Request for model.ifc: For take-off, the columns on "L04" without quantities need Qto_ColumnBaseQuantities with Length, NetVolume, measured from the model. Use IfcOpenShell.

First a look at what the model holds.

```python
import ifcopenshell
import ifcopenshell.util.element
import ifcopenshell.util.unit

model = ifcopenshell.open("model.ifc")
print(model.schema)
for unit_type in ("LENGTHUNIT", "AREAUNIT", "VOLUMEUNIT"):
    print(unit_type, ifcopenshell.util.unit.calculate_unit_scale(model, unit_type))
storey = next(s for s in model.by_type("IfcBuildingStorey") if s.Name == "L04")
columns = [e for e in ifcopenshell.util.element.get_decomposition(storey) if e.is_a("IfcColumn")]
for e in sorted(columns, key=lambda e: e.id()):
    print(e.id(), e.is_a(), e.Name, list(ifcopenshell.util.element.get_psets(e, qtos_only=True)), sep=" | ")
```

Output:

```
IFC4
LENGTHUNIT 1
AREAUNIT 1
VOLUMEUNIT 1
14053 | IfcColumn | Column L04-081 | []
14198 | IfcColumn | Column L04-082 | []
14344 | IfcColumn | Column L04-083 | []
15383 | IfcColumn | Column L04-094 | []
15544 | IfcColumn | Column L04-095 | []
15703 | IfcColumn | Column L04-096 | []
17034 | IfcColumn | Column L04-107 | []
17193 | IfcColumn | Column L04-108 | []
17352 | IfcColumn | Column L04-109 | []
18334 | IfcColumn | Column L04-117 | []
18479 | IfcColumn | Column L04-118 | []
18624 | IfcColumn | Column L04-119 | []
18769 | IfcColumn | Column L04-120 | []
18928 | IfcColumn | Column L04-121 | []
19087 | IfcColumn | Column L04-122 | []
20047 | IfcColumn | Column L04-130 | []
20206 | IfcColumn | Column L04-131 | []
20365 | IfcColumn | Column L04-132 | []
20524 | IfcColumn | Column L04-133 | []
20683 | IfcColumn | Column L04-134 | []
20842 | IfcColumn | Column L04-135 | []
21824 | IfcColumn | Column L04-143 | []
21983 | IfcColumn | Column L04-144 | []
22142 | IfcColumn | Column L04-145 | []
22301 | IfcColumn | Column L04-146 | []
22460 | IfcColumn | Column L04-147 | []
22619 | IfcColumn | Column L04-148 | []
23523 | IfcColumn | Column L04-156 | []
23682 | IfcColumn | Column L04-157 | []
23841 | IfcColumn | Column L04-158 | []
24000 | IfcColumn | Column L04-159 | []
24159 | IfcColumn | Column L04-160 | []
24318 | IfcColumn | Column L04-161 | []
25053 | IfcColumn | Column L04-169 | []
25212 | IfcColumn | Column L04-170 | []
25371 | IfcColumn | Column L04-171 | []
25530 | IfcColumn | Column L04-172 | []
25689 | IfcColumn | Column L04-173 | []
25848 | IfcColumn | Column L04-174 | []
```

```python
import ifcopenshell
import ifcopenshell.api.pset
import ifcopenshell.geom
import ifcopenshell.util.element
import ifcopenshell.util.shape
import ifcopenshell.util.unit

model = ifcopenshell.open("model.ifc")
unit_scale = ifcopenshell.util.unit.calculate_unit_scale(model)
volume_scale = ifcopenshell.util.unit.calculate_unit_scale(model, "VOLUMEUNIT")
settings = ifcopenshell.geom.settings()

storey = next(s for s in model.by_type("IfcBuildingStorey") if s.Name == "L04")
columns = [e for e in ifcopenshell.util.element.get_decomposition(storey) if e.is_a("IfcColumn")]

for e in sorted(columns, key=lambda e: e.id()):
    if ifcopenshell.util.element.get_psets(e, qtos_only=True, should_inherit=False):
        continue
    # Geometry comes back in metres, in the element's own axes.
    shape = ifcopenshell.geom.create_shape(settings, e)
    values = {
        "Length": ifcopenshell.util.shape.get_z(shape.geometry) / unit_scale,
        "NetVolume": ifcopenshell.util.shape.get_volume(shape.geometry) / volume_scale,
    }
    qto = ifcopenshell.api.pset.add_qto(model, product=e, name="Qto_ColumnBaseQuantities")
    ifcopenshell.api.pset.edit_qto(model, qto=qto, properties=values)
    print(e.id(), {k: round(v, 3) for k, v in values.items()})

model.write("model-out.ifc")
```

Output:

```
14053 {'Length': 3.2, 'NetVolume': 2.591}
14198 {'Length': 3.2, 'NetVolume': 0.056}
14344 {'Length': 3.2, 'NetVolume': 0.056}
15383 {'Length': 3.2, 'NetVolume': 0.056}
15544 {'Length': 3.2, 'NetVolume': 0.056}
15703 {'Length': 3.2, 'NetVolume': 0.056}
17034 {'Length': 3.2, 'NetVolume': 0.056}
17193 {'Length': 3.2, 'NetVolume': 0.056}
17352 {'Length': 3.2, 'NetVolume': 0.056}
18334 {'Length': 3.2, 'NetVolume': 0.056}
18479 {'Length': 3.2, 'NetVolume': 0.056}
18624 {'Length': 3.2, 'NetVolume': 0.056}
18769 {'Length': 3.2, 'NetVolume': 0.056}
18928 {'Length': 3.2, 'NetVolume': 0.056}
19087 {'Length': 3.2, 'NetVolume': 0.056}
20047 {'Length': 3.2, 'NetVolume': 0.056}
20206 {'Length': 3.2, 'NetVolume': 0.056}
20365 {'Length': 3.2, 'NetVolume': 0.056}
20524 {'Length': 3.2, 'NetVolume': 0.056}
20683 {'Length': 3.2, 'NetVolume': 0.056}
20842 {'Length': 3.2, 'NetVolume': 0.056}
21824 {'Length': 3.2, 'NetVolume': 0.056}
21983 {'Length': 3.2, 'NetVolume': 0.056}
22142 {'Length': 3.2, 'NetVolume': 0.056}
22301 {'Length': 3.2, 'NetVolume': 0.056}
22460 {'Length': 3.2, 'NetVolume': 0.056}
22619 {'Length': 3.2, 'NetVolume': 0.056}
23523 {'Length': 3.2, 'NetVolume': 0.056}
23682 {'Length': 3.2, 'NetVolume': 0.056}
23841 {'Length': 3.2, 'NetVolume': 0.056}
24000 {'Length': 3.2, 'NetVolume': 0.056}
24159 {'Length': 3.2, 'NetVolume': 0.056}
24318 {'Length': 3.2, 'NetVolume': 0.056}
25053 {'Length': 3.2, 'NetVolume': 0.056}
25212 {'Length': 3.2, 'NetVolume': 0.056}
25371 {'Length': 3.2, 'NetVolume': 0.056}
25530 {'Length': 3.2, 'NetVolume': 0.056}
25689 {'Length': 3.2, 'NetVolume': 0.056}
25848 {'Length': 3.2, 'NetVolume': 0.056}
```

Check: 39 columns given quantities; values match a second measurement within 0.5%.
